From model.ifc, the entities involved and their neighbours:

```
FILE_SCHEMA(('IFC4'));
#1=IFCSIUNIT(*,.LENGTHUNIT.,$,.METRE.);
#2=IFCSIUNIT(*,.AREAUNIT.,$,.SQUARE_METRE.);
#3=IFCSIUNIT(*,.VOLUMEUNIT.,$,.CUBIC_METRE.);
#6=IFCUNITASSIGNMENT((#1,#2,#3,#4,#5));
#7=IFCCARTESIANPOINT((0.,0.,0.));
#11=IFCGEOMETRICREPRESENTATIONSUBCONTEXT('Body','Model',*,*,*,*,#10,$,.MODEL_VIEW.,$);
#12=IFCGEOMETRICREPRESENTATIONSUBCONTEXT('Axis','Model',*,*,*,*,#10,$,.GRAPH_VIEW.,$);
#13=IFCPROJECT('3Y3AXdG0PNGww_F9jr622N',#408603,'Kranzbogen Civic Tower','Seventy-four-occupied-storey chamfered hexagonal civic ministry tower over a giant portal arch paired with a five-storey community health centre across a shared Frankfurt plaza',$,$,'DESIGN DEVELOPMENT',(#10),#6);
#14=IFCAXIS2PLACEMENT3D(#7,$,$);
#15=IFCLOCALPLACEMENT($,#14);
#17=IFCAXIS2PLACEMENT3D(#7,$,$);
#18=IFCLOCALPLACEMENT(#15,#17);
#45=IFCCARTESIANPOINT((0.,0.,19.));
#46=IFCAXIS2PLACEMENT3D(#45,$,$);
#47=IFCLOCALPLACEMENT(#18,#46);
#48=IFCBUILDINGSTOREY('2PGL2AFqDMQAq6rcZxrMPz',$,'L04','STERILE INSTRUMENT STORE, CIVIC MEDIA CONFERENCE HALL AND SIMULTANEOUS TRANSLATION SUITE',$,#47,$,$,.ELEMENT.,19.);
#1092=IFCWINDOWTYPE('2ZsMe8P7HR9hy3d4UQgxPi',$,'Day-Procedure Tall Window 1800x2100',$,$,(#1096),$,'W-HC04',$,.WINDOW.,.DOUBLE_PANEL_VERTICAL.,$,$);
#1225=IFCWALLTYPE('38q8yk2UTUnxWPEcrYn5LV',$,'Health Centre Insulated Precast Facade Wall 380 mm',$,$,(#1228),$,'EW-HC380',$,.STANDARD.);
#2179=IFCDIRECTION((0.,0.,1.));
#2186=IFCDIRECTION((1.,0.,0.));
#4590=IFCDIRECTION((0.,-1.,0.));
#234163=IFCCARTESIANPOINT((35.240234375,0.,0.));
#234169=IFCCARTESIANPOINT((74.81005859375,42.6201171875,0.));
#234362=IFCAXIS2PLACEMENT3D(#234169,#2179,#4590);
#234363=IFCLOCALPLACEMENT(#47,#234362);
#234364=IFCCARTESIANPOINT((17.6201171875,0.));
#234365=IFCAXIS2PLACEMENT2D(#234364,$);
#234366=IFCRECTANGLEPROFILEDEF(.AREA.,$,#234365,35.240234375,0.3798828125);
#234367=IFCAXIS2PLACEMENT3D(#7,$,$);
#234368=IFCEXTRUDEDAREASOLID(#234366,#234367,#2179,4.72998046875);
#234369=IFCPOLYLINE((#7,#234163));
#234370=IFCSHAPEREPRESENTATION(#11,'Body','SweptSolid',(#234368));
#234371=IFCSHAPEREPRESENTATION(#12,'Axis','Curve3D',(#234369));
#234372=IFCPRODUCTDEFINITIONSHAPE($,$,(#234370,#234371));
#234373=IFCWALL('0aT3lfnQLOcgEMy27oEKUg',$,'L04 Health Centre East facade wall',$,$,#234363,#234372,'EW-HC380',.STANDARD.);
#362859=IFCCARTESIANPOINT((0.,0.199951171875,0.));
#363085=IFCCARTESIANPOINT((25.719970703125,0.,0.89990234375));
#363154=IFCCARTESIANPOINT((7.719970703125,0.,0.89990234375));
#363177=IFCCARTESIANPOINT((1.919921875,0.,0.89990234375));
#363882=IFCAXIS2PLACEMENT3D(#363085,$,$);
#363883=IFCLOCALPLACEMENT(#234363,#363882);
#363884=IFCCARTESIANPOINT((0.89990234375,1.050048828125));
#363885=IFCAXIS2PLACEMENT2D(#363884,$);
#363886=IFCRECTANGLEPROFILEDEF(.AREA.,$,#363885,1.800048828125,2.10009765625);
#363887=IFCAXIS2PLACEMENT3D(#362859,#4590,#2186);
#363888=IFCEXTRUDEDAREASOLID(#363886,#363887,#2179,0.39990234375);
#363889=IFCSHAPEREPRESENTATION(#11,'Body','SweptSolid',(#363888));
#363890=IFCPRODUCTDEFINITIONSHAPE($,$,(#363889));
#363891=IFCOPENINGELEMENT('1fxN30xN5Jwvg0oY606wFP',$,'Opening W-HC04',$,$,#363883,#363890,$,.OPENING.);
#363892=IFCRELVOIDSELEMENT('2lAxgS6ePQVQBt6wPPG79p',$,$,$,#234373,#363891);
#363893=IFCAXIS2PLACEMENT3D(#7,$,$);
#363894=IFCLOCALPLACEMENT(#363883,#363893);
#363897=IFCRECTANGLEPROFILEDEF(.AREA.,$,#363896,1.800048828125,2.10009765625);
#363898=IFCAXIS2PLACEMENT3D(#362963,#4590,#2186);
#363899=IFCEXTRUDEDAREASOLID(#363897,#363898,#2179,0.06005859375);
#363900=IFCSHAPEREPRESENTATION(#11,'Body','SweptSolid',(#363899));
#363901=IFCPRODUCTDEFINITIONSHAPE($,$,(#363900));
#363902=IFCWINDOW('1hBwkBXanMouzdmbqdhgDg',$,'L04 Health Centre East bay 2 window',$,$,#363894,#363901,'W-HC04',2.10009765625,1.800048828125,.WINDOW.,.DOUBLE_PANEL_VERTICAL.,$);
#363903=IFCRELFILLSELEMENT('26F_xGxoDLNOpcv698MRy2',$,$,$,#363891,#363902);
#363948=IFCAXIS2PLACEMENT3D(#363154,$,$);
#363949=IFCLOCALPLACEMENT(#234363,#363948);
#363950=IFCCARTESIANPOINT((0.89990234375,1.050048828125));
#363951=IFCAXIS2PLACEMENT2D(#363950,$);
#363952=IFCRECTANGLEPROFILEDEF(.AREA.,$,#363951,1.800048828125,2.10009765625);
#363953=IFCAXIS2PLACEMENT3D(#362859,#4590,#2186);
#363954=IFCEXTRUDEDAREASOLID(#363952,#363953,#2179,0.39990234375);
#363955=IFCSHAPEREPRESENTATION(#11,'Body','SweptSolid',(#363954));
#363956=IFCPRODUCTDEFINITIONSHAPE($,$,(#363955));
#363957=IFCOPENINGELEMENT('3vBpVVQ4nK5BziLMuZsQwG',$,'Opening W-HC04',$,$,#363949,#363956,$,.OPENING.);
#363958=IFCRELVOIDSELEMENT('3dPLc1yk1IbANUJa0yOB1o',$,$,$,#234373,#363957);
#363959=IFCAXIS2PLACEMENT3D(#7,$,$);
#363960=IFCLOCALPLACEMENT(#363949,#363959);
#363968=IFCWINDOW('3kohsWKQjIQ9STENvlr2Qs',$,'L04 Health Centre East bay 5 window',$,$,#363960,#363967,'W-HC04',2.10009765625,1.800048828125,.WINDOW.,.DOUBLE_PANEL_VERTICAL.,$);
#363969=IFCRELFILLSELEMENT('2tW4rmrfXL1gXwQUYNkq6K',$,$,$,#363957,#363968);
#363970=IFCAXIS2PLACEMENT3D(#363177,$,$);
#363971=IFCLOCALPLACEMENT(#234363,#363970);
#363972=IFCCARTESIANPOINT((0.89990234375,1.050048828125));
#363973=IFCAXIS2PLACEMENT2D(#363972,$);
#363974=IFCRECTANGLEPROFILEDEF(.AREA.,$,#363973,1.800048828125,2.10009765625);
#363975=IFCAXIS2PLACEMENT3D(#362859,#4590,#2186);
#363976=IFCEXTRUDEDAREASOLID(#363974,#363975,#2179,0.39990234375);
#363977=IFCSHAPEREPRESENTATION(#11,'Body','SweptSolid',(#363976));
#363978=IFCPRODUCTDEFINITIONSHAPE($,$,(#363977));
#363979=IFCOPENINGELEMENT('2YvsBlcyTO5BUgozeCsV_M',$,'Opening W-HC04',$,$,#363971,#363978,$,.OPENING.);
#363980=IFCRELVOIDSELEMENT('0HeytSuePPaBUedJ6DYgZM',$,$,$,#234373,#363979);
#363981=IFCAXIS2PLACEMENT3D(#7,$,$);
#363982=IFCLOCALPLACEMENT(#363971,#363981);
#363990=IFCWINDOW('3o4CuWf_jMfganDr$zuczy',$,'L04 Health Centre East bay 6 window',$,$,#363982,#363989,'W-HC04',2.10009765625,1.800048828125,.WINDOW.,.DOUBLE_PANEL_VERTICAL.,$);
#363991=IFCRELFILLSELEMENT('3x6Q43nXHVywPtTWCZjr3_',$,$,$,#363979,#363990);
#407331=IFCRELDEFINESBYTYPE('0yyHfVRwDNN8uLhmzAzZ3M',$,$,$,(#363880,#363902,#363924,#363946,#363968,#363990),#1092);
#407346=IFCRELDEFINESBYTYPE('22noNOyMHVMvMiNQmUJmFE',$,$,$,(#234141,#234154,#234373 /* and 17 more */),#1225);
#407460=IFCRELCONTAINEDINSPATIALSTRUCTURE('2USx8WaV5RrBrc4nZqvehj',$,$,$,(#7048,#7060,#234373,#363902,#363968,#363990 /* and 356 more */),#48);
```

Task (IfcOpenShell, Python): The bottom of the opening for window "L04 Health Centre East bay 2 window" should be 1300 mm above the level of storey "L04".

```python
import numpy as np
import ifcopenshell
import ifcopenshell.api.geometry
import ifcopenshell.geom
import ifcopenshell.util.element
import ifcopenshell.util.placement
import ifcopenshell.util.shape
import ifcopenshell.util.unit

model = ifcopenshell.open("model.ifc")
unit_scale = ifcopenshell.util.unit.calculate_unit_scale(model)

window = model.by_guid("1hBwkBXanMouzdmbqdhgDg")
opening = window.FillsVoids[0].RelatingOpeningElement
storey = ifcopenshell.util.element.get_container(window, ifc_class="IfcBuildingStorey")
level = ifcopenshell.util.placement.get_local_placement(storey.ObjectPlacement)[2, 3]

# The opening's origin need not be at the sill, so measure its lowest point.
shape = ifcopenshell.geom.create_shape(ifcopenshell.geom.settings(), opening)
bottom = ifcopenshell.util.shape.get_shape_bottom_elevation(shape, shape.geometry) / unit_scale
dz = level + 1.3 / unit_scale - bottom

shift = np.array([0.0, 0.0, dz])
# The window is placed relative to its opening, so it follows when the opening moves.
matrix = ifcopenshell.util.placement.get_local_placement(opening.ObjectPlacement)
matrix[:3, 3] += shift
ifcopenshell.api.geometry.edit_object_placement(
    model, product=opening, matrix=matrix, is_si=False, should_transform_children=True
)

print(f"moved by {dz * unit_scale:+.3f} m")

model.write("model_updated.ifc")
```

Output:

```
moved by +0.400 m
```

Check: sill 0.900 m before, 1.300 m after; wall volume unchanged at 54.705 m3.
